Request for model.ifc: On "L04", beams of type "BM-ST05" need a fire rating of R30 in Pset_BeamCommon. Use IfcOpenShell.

First a look at what the model holds.

```python
import ifcopenshell
import ifcopenshell.util.element

model = ifcopenshell.open("model.ifc")
print(model.schema)
storey = next(s for s in model.by_type("IfcBuildingStorey") if s.Name == "L04")
beams = [e for e in ifcopenshell.util.element.get_decomposition(storey) if e.is_a("IfcBeam")]
seen = {}
for e in beams:
    element_type = ifcopenshell.util.element.get_type(e)
    key = (element_type.Name if element_type != e and element_type else None, ifcopenshell.util.element.get_pset(e, "Pset_BeamCommon", "FireRating"))
    seen[key] = seen.get(key, 0) + 1
for (name, value), count in sorted(seen.items(), key=str):
    print(count, "x", name, "|", value)
```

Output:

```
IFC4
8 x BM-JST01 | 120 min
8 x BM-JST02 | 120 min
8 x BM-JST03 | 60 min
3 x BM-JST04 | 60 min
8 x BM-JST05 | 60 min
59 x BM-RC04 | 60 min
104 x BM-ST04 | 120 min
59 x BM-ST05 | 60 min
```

```python
import ifcopenshell
import ifcopenshell.api.pset
import ifcopenshell.util.element

model = ifcopenshell.open("model.ifc")

storey = next(s for s in model.by_type("IfcBuildingStorey") if s.Name == "L04")
beams = [e for e in ifcopenshell.util.element.get_decomposition(storey) if e.is_a("IfcBeam")]

count = 0
for e in beams:
    element_type = ifcopenshell.util.element.get_type(e)
    if element_type in (None, e) or element_type.Name != "BM-ST05":
        continue
    # add_pset returns the element's existing set when there is one.
    pset = ifcopenshell.api.pset.add_pset(model, product=e, name="Pset_BeamCommon")
    ifcopenshell.api.pset.edit_pset(model, pset=pset, properties={"FireRating": "R30"})
    count += 1

print(count, "beams updated")

model.write("model_updated.ifc")
```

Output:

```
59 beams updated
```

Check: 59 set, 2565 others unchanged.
